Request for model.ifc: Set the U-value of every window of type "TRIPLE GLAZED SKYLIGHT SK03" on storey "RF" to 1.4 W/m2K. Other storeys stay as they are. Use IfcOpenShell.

First a look at what the model holds.

```python
import ifcopenshell
import ifcopenshell.util.element

model = ifcopenshell.open("model.ifc")
print(model.schema)
storey = next(s for s in model.by_type("IfcBuildingStorey") if s.Name == "RF")
windows = [e for e in ifcopenshell.util.element.get_decomposition(storey) if e.is_a("IfcWindow")]
seen = {}
for e in windows:
    element_type = ifcopenshell.util.element.get_type(e)
    key = (element_type.Name if element_type != e and element_type else None, ifcopenshell.util.element.get_pset(e, "Pset_WindowCommon", "ThermalTransmittance"))
    seen[key] = seen.get(key, 0) + 1
for (name, value), count in sorted(seen.items(), key=str):
    print(count, "x", name, "|", value)
```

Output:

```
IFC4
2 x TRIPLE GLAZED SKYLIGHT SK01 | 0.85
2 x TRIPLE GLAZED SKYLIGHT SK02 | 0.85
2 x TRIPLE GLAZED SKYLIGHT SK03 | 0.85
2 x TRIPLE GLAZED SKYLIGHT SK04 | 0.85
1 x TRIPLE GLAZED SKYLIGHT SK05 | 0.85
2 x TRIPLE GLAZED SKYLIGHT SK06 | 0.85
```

```python
import ifcopenshell
import ifcopenshell.api.pset
import ifcopenshell.util.element

model = ifcopenshell.open("model.ifc")

storey = next(s for s in model.by_type("IfcBuildingStorey") if s.Name == "RF")
windows = [e for e in ifcopenshell.util.element.get_decomposition(storey) if e.is_a("IfcWindow")]

count = 0
for e in windows:
    element_type = ifcopenshell.util.element.get_type(e)
    if element_type in (None, e) or element_type.Name != "TRIPLE GLAZED SKYLIGHT SK03":
        continue
    # add_pset returns the element's existing set when there is one.
    pset = ifcopenshell.api.pset.add_pset(model, product=e, name="Pset_WindowCommon")
    ifcopenshell.api.pset.edit_pset(model, pset=pset, properties={"ThermalTransmittance": 1.4})
    count += 1

print(count, "windows updated")

model.write("model_v2.ifc")
```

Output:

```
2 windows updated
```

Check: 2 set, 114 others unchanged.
